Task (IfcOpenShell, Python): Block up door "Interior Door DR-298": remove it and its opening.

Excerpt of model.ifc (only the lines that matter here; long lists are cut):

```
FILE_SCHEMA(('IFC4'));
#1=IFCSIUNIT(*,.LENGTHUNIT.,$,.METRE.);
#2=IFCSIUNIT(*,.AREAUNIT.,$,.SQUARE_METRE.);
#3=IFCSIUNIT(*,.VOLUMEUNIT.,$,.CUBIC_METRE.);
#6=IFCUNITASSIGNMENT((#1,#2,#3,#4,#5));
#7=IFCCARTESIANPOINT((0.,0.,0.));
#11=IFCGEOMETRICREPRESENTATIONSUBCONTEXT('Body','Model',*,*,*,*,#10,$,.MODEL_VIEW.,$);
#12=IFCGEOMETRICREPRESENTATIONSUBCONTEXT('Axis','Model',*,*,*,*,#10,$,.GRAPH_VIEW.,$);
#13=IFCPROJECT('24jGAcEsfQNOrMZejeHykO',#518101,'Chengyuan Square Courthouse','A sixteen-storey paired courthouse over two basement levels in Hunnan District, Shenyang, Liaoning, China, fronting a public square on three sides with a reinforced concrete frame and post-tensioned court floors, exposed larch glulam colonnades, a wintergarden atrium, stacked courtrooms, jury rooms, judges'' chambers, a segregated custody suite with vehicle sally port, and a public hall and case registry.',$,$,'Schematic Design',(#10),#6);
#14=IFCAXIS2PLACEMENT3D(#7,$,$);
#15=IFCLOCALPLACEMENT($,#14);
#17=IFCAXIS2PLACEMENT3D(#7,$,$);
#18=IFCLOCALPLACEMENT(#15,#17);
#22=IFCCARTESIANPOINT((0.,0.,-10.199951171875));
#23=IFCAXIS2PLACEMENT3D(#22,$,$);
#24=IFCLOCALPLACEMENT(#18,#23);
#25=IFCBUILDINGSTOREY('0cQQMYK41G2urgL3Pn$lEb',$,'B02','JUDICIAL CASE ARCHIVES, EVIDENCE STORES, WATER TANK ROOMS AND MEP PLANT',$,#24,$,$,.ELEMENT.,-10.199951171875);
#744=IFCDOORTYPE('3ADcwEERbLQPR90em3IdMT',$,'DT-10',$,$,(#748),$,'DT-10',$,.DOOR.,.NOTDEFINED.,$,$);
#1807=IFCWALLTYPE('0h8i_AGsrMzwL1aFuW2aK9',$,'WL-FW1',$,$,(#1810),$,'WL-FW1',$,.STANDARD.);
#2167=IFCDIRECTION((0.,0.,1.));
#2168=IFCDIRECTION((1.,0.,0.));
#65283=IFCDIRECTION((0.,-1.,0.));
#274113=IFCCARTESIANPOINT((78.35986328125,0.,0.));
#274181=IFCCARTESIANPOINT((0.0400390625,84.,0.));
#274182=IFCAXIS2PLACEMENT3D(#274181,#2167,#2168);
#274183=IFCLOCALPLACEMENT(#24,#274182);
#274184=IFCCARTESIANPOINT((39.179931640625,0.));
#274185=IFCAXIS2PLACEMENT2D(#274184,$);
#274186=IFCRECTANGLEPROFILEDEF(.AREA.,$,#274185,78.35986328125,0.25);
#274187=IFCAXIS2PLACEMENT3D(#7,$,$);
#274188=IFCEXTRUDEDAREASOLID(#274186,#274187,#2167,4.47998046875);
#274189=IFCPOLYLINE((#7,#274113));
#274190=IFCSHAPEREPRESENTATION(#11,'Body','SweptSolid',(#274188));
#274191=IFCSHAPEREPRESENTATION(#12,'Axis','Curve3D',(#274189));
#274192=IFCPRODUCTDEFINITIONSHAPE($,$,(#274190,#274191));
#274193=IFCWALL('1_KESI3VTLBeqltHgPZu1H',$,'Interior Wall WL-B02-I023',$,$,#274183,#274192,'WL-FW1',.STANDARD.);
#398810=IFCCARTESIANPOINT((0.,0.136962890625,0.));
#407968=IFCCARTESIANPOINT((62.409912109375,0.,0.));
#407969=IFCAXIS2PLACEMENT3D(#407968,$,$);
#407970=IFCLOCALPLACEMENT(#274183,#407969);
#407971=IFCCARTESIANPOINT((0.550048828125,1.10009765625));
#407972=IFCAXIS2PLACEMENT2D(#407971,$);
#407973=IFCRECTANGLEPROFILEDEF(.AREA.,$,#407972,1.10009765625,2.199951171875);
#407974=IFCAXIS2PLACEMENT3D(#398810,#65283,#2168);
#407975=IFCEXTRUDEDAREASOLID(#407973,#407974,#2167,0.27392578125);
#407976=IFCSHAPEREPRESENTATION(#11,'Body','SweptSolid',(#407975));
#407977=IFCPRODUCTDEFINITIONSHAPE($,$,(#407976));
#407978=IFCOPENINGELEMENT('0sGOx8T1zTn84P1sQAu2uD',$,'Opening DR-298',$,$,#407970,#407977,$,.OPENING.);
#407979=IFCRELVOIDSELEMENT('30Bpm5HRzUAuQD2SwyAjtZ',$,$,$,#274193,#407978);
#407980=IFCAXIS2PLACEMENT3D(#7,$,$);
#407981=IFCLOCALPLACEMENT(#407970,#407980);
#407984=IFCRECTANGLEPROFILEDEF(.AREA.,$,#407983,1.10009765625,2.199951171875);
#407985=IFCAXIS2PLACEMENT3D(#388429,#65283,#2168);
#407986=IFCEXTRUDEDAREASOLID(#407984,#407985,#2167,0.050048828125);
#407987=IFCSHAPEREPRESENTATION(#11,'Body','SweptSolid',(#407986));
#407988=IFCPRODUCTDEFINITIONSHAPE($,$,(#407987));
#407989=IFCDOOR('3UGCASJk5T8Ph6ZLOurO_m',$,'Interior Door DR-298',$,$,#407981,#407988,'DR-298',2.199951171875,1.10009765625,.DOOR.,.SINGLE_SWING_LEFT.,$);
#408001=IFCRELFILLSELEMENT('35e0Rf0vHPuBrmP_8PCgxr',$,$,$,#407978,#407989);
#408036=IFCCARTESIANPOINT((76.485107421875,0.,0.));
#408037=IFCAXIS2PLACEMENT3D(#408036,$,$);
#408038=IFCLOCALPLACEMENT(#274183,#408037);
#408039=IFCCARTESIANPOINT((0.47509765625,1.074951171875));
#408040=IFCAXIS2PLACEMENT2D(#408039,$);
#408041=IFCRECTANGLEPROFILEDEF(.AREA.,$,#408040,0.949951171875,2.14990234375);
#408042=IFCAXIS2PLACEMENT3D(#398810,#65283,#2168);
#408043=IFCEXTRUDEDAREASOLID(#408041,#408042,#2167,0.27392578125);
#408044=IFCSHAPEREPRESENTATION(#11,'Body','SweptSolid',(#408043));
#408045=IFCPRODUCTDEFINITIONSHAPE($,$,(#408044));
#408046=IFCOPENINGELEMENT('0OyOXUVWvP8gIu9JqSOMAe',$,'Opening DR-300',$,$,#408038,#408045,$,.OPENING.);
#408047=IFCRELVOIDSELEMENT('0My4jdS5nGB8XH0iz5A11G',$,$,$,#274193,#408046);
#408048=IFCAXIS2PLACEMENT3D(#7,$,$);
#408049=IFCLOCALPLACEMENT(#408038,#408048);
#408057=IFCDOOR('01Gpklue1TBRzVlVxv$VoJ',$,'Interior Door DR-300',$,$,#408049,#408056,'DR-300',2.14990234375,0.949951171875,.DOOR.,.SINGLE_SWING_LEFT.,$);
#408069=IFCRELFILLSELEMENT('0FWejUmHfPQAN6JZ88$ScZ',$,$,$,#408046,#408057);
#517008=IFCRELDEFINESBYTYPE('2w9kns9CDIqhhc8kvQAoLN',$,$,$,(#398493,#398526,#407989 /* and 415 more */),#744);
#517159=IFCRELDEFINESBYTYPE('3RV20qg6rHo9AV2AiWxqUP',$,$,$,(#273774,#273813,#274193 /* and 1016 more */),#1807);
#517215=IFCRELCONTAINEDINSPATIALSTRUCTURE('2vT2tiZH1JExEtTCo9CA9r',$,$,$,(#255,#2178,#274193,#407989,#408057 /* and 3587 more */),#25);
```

```python
import ifcopenshell
import ifcopenshell.api.feature
import ifcopenshell.api.root
import ifcopenshell.geom
import ifcopenshell.util.shape

model = ifcopenshell.open("model.ifc")
settings = ifcopenshell.geom.settings()


def volume(element):
    """Net volume in cubic metres, openings subtracted."""
    shape = ifcopenshell.geom.create_shape(settings, element)
    return ifcopenshell.util.shape.get_volume(shape.geometry)


door = model.by_guid("3UGCASJk5T8Ph6ZLOurO_m")
opening = door.FillsVoids[0].RelatingOpeningElement
wall = opening.VoidsElements[0].RelatingBuildingElement
before = volume(wall)

ifcopenshell.api.root.remove_product(model, product=door)
ifcopenshell.api.feature.remove_feature(model, feature=opening)

after = volume(wall)

print(f"wall volume {before:.3f} -> {after:.3f} m3")

model.write("model_updated.ifc")
```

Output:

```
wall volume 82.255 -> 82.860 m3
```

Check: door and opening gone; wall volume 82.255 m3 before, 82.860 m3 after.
